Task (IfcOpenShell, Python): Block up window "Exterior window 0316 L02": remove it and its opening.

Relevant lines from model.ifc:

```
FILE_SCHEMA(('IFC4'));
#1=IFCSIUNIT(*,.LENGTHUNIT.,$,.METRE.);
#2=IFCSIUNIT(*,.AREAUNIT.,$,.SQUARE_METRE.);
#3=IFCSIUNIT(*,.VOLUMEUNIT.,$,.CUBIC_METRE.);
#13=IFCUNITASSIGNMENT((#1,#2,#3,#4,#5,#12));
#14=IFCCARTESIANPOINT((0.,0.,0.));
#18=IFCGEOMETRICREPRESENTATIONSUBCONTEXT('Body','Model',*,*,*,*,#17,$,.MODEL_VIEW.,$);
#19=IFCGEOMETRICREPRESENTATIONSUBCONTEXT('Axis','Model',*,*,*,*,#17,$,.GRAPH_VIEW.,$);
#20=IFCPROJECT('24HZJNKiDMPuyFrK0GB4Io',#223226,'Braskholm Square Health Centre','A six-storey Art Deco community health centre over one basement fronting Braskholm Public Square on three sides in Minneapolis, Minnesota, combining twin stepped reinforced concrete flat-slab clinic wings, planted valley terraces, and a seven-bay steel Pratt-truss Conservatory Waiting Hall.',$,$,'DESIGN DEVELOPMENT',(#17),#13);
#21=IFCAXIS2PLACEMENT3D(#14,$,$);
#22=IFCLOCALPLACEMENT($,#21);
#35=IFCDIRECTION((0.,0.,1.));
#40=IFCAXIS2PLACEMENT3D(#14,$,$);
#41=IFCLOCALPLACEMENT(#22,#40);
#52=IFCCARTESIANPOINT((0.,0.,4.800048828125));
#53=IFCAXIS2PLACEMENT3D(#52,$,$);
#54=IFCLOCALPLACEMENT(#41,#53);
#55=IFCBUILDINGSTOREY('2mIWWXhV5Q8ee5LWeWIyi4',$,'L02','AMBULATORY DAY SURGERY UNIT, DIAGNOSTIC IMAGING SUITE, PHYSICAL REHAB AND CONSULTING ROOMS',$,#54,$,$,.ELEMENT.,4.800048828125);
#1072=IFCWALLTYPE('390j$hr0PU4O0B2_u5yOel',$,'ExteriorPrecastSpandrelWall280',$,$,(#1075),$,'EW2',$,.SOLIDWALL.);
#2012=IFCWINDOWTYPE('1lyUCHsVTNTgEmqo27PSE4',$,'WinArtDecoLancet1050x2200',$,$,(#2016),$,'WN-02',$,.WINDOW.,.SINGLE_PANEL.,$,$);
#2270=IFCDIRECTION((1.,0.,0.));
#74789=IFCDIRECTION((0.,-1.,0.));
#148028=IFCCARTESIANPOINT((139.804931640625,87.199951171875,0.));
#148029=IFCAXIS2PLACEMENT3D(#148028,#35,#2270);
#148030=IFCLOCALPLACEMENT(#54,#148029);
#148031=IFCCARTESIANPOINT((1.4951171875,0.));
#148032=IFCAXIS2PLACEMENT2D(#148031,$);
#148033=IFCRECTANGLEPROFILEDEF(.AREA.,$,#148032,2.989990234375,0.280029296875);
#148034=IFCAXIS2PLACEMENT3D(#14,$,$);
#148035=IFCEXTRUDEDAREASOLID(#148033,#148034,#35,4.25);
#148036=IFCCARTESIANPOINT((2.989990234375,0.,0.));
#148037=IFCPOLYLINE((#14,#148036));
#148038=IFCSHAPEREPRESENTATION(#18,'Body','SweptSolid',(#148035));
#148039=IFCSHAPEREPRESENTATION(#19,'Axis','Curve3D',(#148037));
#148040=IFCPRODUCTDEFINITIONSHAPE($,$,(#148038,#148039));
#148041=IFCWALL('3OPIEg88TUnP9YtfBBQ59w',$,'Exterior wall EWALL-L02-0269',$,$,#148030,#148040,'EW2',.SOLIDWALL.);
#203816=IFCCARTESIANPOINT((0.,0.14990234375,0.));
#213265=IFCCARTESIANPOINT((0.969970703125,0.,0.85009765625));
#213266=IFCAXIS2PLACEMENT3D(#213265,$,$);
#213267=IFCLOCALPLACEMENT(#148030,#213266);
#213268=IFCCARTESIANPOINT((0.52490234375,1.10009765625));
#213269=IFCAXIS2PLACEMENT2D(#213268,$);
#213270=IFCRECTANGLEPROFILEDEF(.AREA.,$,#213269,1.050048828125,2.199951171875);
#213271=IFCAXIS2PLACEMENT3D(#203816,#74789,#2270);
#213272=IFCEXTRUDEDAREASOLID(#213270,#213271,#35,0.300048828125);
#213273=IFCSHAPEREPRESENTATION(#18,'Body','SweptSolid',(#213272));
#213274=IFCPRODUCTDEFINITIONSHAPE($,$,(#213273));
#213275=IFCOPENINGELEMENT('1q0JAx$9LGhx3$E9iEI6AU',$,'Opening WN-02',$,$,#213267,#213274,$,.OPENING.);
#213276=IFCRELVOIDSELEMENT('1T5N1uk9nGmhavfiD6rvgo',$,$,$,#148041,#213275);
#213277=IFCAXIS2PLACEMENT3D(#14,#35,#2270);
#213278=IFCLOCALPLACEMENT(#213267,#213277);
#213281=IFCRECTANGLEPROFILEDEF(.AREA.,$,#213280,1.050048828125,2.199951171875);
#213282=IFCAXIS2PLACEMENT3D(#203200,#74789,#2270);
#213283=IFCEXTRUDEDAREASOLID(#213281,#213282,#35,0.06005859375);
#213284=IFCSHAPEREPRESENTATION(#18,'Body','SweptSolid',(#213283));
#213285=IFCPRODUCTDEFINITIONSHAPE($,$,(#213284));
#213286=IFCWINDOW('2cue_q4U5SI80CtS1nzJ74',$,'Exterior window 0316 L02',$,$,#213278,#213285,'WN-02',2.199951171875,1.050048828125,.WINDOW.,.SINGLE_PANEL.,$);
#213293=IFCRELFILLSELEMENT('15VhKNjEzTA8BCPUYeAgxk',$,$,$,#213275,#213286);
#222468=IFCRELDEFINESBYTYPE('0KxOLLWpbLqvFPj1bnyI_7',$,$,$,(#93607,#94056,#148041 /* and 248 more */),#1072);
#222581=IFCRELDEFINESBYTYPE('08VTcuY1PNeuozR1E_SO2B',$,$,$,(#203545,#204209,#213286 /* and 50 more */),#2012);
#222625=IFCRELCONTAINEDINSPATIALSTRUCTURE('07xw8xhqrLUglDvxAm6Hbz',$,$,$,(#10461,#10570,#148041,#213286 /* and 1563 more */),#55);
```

```python
import ifcopenshell
import ifcopenshell.api.feature
import ifcopenshell.api.root
import ifcopenshell.geom
import ifcopenshell.util.shape

model = ifcopenshell.open("model.ifc")
settings = ifcopenshell.geom.settings()


def volume(element):
    """Net volume in cubic metres, openings subtracted."""
    shape = ifcopenshell.geom.create_shape(settings, element)
    return ifcopenshell.util.shape.get_volume(shape.geometry)


window = model.by_guid("2cue_q4U5SI80CtS1nzJ74")
opening = window.FillsVoids[0].RelatingOpeningElement
wall = opening.VoidsElements[0].RelatingBuildingElement
before = volume(wall)

ifcopenshell.api.root.remove_product(model, product=window)
ifcopenshell.api.feature.remove_feature(model, feature=opening)

after = volume(wall)

print(f"wall volume {before:.3f} -> {after:.3f} m3")

model.write("model_v2.ifc")
```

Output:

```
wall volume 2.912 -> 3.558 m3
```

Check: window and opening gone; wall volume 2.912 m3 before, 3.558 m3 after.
